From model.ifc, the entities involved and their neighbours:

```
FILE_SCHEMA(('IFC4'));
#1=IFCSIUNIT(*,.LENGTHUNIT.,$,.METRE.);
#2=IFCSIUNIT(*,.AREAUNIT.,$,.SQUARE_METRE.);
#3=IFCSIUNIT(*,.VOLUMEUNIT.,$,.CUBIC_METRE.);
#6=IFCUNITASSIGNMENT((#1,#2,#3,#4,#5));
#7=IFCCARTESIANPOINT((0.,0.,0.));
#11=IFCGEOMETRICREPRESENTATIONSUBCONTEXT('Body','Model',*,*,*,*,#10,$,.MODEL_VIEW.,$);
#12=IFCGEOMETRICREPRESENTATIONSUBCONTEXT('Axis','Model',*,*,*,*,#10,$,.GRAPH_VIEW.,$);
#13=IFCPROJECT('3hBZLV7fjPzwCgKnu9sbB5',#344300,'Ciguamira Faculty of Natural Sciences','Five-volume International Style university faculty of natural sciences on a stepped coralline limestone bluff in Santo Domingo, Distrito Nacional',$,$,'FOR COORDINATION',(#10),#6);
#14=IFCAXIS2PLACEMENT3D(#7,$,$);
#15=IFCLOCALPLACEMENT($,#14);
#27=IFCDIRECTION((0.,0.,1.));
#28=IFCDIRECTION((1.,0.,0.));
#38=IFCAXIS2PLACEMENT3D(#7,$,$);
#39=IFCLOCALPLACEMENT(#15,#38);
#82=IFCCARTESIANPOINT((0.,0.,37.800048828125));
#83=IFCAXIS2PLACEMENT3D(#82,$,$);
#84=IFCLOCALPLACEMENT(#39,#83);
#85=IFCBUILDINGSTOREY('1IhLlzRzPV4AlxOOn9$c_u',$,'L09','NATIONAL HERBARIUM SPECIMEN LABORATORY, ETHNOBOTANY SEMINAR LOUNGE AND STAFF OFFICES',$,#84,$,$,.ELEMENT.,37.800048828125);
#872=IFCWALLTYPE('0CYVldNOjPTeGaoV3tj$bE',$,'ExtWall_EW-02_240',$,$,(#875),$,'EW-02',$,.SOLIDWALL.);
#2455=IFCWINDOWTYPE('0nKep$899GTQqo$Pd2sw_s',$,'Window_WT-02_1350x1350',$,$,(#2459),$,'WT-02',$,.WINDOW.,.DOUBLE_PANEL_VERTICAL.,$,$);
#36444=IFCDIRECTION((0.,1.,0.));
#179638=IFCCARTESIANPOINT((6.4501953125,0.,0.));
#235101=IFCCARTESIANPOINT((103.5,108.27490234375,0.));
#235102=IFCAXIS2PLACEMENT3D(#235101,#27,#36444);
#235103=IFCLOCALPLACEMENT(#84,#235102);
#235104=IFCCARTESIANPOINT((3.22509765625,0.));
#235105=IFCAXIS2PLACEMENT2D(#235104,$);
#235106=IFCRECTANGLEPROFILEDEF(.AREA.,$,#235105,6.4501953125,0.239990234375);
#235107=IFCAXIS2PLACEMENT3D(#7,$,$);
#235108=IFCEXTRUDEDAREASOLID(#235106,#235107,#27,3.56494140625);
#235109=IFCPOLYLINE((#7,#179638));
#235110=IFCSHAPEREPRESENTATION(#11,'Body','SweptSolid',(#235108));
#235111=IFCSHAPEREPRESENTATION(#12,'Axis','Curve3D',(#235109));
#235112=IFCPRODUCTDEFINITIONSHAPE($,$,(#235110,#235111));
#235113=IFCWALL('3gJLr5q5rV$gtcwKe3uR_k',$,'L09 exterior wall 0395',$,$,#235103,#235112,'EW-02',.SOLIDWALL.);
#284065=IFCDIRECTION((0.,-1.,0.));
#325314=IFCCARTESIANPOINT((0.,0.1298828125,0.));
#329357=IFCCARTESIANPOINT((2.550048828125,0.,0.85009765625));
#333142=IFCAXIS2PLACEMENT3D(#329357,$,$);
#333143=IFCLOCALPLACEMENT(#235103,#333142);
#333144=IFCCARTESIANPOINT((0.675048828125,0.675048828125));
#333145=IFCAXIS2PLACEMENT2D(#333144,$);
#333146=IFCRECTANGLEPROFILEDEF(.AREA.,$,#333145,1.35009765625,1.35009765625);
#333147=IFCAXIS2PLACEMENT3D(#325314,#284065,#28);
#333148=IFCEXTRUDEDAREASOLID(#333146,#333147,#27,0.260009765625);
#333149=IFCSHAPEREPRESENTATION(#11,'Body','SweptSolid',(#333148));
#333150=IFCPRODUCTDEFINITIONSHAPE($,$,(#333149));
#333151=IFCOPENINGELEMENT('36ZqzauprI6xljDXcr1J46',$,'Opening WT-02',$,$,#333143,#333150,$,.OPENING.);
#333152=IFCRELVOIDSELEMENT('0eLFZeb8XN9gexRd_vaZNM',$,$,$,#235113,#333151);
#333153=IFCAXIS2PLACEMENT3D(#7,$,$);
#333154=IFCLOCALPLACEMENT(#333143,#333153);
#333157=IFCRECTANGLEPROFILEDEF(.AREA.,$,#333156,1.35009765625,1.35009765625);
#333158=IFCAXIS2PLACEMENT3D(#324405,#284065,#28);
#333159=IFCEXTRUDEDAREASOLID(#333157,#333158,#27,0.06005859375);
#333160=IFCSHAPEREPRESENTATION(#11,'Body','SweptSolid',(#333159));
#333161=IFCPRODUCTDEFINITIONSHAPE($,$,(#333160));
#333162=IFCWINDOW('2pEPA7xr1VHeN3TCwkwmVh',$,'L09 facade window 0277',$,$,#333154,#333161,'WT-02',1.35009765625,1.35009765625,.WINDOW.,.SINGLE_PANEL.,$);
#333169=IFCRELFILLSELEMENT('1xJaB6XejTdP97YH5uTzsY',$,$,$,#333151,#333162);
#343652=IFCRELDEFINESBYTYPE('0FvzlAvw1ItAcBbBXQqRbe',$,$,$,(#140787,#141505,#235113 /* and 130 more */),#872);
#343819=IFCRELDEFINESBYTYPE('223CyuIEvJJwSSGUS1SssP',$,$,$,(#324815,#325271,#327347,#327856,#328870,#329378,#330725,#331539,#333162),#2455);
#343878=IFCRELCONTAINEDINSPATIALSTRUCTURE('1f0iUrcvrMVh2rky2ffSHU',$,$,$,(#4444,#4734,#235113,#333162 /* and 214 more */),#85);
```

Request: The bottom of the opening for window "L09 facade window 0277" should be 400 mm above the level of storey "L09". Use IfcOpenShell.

```python
import numpy as np
import ifcopenshell
import ifcopenshell.api.geometry
import ifcopenshell.geom
import ifcopenshell.util.element
import ifcopenshell.util.placement
import ifcopenshell.util.shape
import ifcopenshell.util.unit

model = ifcopenshell.open("model.ifc")
unit_scale = ifcopenshell.util.unit.calculate_unit_scale(model)

window = model.by_id(333162)
opening = window.FillsVoids[0].RelatingOpeningElement
storey = ifcopenshell.util.element.get_container(window, ifc_class="IfcBuildingStorey")
level = ifcopenshell.util.placement.get_local_placement(storey.ObjectPlacement)[2, 3]

# The opening's origin need not be at the sill, so measure its lowest point.
shape = ifcopenshell.geom.create_shape(ifcopenshell.geom.settings(), opening)
bottom = ifcopenshell.util.shape.get_shape_bottom_elevation(shape, shape.geometry) / unit_scale
dz = level + 0.4 - bottom

shift = np.array([0.0, 0.0, dz])
# The window is placed relative to its opening, so it follows when the opening moves.
matrix = ifcopenshell.util.placement.get_local_placement(opening.ObjectPlacement)
matrix[:3, 3] += shift
ifcopenshell.api.geometry.edit_object_placement(
    model, product=opening, matrix=matrix, is_si=False, should_transform_children=True
)

print(f"moved by {dz * unit_scale:+.3f} m")

model.write("model-out.ifc")
```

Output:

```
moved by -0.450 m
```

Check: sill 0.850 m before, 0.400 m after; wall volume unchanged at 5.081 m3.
